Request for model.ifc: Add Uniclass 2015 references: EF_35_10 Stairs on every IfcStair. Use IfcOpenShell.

First a look at what the model holds.

```python
import ifcopenshell

model = ifcopenshell.open("model.ifc")
print(model.schema)
print("classifications:", [c.Name for c in model.by_type("IfcClassification")])
for ifc_class in ("IfcDoor", "IfcRoof", "IfcStair", "IfcWall", "IfcWindow"):
    print(ifc_class, len(model.by_type(ifc_class)))
```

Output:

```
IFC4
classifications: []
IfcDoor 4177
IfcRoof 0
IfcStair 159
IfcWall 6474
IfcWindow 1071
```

```python
import ifcopenshell
import ifcopenshell.api.classification

model = ifcopenshell.open("model.ifc")

system = ifcopenshell.api.classification.add_classification(model, classification="Uniclass 2015")

codes = {
    "IfcStair": ("EF_35_10", "Stairs"),
}
for ifc_class, (code, name) in codes.items():
    products = model.by_type(ifc_class)
    ifcopenshell.api.classification.add_reference(
        model, products=products, classification=system, identification=code, name=name
    )
    print(code, len(products))

model.write("model-out.ifc")
```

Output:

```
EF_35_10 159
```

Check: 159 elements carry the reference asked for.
